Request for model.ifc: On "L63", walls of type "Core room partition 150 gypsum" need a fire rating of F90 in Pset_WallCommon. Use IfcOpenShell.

First a look at what the model holds.

```python
import ifcopenshell
import ifcopenshell.util.element

model = ifcopenshell.open("model.ifc")
print(model.schema)
storey = next(s for s in model.by_type("IfcBuildingStorey") if s.Name == "L63")
walls = [e for e in ifcopenshell.util.element.get_decomposition(storey) if e.is_a("IfcWall")]
seen = {}
for e in walls:
    element_type = ifcopenshell.util.element.get_type(e)
    key = (element_type.Name if element_type != e and element_type else None, ifcopenshell.util.element.get_pset(e, "Pset_WallCommon", "FireRating"))
    seen[key] = seen.get(key, 0) + 1
for (name, value), count in sorted(seen.items(), key=str):
    print(count, "x", name, "|", value)
```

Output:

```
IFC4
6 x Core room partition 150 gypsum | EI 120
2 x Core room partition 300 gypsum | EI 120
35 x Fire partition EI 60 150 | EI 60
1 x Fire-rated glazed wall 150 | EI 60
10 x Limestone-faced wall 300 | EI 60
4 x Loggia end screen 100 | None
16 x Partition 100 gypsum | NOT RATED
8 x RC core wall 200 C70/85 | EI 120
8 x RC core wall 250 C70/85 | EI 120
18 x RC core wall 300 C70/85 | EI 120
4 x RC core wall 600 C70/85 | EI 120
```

```python
import ifcopenshell
import ifcopenshell.api.pset
import ifcopenshell.util.element

model = ifcopenshell.open("model.ifc")

storey = next(s for s in model.by_type("IfcBuildingStorey") if s.Name == "L63")
walls = [e for e in ifcopenshell.util.element.get_decomposition(storey) if e.is_a("IfcWall")]

count = 0
for e in walls:
    element_type = ifcopenshell.util.element.get_type(e)
    if element_type in (None, e) or element_type.Name != "Core room partition 150 gypsum":
        continue
    found = ifcopenshell.util.element.get_pset(e, "Pset_WallCommon", should_inherit=False)
    if found:
        pset = model.by_id(found["id"])
        if len(ifcopenshell.util.element.get_elements_by_pset(pset)) > 1:
            pset = ifcopenshell.api.pset.unshare_pset(model, products=[e], pset=pset)[0]
    else:
        pset = ifcopenshell.api.pset.add_pset(model, product=e, name="Pset_WallCommon")
    ifcopenshell.api.pset.edit_pset(model, pset=pset, properties={"FireRating": "F90"})
    count += 1

print(count, "walls updated")

model.write("model_rev.ifc")
```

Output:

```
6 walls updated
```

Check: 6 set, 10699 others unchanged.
